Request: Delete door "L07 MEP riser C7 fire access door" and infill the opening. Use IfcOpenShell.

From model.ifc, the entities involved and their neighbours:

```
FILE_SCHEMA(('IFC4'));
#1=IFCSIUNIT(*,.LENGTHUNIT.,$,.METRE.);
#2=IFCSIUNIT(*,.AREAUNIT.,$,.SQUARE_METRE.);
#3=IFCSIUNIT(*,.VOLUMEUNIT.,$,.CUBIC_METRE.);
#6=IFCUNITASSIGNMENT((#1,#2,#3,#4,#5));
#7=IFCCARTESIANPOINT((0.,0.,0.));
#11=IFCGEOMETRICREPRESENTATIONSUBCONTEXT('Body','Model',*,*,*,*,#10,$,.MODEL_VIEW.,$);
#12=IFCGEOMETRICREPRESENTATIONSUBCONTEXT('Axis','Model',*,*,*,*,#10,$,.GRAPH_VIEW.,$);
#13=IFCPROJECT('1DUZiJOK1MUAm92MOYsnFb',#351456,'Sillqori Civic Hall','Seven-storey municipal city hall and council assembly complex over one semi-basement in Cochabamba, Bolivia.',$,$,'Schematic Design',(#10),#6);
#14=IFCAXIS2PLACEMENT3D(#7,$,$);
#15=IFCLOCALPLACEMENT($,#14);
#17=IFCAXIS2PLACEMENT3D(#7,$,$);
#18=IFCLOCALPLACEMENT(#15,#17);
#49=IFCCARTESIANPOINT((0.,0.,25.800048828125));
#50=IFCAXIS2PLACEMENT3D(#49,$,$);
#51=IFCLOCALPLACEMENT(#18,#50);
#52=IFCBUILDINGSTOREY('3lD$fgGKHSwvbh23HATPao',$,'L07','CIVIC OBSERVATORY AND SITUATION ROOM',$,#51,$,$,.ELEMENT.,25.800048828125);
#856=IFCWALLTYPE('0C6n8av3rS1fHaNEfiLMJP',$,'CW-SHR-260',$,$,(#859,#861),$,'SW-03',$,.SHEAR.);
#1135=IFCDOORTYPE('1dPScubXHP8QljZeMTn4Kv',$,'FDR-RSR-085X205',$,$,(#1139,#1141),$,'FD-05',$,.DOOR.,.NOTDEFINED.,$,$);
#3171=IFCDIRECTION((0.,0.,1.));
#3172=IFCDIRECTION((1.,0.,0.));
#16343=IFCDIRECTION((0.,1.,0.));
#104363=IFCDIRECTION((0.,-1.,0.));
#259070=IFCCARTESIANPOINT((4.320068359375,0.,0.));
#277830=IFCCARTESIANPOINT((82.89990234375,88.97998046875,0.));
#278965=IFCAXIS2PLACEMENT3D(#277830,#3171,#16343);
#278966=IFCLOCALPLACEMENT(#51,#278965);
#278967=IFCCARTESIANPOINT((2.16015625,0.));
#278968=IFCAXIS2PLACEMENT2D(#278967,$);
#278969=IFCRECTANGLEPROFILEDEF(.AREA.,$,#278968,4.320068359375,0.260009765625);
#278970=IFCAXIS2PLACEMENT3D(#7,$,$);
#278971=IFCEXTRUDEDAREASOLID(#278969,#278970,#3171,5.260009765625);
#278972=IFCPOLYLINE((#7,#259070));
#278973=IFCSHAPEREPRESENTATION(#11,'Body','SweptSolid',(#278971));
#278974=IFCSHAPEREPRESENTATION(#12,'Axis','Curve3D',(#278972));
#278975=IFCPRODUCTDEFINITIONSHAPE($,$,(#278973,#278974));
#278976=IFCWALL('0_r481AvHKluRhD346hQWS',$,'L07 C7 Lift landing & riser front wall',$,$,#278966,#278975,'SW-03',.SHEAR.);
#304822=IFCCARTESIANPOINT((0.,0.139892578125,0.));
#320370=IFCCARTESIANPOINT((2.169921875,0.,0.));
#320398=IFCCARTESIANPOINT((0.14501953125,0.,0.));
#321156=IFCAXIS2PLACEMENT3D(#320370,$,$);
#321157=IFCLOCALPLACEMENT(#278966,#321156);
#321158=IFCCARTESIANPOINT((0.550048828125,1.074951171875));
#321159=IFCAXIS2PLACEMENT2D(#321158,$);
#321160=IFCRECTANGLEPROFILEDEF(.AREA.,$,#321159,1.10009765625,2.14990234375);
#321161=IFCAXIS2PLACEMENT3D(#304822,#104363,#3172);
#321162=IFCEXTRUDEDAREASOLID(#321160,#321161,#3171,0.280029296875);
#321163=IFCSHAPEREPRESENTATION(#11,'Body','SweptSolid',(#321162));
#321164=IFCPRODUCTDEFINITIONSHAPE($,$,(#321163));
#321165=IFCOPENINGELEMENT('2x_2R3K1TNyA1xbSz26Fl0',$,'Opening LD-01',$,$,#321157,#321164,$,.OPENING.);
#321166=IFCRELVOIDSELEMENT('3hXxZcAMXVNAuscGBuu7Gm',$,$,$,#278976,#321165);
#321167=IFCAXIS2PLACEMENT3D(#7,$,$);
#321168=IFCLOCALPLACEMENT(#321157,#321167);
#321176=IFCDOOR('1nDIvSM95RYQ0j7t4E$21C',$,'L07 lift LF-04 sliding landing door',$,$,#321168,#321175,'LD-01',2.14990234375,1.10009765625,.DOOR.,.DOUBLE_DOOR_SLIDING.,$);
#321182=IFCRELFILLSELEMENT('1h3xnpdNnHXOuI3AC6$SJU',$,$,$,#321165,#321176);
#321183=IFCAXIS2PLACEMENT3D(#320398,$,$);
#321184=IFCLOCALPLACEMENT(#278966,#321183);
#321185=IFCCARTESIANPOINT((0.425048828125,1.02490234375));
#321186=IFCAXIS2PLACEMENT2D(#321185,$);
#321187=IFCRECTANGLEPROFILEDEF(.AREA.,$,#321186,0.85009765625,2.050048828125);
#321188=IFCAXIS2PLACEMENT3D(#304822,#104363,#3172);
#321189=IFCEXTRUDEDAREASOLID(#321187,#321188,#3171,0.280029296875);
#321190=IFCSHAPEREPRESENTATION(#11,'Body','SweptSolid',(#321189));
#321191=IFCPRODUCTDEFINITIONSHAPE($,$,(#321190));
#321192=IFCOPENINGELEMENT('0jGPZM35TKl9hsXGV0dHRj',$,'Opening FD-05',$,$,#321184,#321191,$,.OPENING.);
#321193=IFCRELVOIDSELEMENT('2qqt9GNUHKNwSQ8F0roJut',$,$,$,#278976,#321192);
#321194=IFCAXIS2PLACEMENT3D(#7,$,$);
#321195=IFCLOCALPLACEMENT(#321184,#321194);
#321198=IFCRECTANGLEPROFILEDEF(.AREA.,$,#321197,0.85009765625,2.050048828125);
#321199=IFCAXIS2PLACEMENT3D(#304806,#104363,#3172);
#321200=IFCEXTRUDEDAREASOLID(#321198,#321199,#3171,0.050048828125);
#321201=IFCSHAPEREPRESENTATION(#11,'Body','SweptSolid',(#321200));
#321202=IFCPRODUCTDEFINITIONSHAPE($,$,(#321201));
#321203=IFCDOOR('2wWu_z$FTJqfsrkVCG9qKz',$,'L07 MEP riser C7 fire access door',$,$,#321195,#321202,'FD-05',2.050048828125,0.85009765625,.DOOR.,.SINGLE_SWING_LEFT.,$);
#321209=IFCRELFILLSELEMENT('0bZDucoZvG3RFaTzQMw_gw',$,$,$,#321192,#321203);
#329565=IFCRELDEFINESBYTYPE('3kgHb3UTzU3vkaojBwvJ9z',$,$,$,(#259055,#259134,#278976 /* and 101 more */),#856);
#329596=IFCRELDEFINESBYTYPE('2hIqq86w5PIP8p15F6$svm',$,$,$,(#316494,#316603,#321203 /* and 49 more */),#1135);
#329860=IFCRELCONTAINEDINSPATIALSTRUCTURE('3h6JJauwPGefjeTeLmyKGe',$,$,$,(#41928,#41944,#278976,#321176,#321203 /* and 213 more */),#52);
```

```python
import ifcopenshell
import ifcopenshell.api.feature
import ifcopenshell.api.root
import ifcopenshell.geom
import ifcopenshell.util.shape

model = ifcopenshell.open("model.ifc")
settings = ifcopenshell.geom.settings()


def volume(element):
    """Net volume in cubic metres, openings subtracted."""
    shape = ifcopenshell.geom.create_shape(settings, element)
    return ifcopenshell.util.shape.get_volume(shape.geometry)


door = model.by_id(321203)
opening = door.FillsVoids[0].RelatingOpeningElement
wall = opening.VoidsElements[0].RelatingBuildingElement
before = volume(wall)

ifcopenshell.api.root.remove_product(model, product=door)
ifcopenshell.api.feature.remove_feature(model, feature=opening)

after = volume(wall)

print(f"wall volume {before:.3f} -> {after:.3f} m3")

model.write("model_edited.ifc")
```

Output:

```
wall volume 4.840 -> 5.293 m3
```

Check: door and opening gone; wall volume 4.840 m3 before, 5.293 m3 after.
